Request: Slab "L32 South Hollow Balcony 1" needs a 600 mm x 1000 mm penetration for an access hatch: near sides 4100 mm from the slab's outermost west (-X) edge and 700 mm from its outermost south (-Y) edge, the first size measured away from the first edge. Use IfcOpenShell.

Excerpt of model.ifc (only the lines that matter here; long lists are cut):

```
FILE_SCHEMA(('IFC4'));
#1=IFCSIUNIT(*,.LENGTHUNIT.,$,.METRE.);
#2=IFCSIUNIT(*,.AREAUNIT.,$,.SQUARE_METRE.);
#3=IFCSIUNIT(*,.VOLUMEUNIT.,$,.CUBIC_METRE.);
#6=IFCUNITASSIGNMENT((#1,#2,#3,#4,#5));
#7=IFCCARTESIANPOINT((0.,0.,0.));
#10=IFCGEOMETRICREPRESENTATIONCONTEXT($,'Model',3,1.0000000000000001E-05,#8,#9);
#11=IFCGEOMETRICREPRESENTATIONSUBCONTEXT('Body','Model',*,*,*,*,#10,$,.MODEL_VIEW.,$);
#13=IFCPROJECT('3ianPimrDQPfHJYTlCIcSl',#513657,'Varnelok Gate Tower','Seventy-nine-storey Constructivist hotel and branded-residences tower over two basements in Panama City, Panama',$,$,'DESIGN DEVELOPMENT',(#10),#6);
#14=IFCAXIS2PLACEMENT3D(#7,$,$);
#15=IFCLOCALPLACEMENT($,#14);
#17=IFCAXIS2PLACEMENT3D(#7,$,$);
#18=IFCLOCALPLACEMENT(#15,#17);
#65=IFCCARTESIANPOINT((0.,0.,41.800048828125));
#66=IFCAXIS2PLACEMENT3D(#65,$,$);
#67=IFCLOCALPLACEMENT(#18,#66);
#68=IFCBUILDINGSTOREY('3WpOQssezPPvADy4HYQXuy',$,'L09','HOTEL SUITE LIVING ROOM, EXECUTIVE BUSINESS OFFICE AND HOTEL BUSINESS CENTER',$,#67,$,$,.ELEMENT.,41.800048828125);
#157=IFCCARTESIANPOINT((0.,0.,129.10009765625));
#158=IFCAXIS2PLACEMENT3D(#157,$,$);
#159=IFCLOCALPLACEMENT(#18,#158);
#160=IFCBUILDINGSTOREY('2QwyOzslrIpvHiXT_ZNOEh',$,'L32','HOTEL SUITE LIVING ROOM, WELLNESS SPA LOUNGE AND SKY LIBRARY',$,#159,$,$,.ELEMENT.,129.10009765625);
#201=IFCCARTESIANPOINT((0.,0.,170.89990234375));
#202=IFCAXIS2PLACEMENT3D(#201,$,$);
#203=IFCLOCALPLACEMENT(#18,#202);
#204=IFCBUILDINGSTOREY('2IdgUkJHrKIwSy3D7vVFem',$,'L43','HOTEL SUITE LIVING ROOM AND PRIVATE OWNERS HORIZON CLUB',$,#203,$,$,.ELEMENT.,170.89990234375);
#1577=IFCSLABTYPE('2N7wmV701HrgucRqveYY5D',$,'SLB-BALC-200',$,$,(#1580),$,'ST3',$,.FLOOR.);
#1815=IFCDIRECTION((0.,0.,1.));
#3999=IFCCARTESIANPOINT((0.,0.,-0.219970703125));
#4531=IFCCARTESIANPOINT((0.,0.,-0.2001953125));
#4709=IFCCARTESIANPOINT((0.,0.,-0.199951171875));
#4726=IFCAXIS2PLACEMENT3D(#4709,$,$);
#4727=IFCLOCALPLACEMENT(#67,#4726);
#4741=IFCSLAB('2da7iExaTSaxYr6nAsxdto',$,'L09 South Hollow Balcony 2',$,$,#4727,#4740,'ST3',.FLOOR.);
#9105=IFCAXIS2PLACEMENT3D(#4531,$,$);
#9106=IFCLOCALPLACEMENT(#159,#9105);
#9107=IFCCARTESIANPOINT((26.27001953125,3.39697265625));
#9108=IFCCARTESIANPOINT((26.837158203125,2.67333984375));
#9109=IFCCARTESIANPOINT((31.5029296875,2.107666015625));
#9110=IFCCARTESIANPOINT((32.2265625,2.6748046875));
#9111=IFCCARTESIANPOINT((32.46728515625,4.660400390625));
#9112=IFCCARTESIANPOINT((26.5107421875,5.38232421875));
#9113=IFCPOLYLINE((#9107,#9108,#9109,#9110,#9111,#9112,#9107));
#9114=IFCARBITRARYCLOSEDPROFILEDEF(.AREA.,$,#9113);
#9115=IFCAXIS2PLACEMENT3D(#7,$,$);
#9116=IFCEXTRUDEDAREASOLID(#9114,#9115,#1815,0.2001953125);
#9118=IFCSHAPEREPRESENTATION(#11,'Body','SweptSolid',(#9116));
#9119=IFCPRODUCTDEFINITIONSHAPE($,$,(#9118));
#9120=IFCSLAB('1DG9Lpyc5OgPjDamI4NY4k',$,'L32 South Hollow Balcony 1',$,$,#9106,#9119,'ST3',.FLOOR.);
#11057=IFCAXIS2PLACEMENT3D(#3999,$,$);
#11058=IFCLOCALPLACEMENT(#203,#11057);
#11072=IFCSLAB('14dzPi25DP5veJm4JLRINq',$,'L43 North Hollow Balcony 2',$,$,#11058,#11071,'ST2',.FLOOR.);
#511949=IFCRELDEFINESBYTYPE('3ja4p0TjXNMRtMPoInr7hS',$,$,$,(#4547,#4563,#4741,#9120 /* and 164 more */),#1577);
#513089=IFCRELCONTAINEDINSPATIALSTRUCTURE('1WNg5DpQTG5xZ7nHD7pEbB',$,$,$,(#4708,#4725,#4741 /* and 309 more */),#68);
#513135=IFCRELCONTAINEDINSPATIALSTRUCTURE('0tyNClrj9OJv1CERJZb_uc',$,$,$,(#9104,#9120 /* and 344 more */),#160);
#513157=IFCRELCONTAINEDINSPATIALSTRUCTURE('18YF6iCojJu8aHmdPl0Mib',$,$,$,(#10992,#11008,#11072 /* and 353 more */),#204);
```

```python
import numpy as np
import ifcopenshell
import ifcopenshell.api.feature
import ifcopenshell.api.geometry
import ifcopenshell.api.root
import ifcopenshell.geom
import ifcopenshell.util.placement
import ifcopenshell.util.representation
import ifcopenshell.util.shape
import ifcopenshell.util.unit

model = ifcopenshell.open("model.ifc")
unit_scale = ifcopenshell.util.unit.calculate_unit_scale(model)
settings = ifcopenshell.geom.settings()


def volume(element):
    """Net volume in cubic metres, openings subtracted."""
    shape = ifcopenshell.geom.create_shape(settings, element)
    return ifcopenshell.util.shape.get_volume(shape.geometry)


slab = model.by_guid("1DG9Lpyc5OgPjDamI4NY4k")
before = volume(slab)

# Extent in the slab's own axes, in metres. The edges named are its -X and -Y sides.
slab_shape = ifcopenshell.geom.create_shape(settings, slab)
vertices = ifcopenshell.util.shape.get_vertices(slab_shape.geometry)
x_min, y_min, bottom = vertices.min(axis=0)
top = vertices[:, 2].max()

opening = ifcopenshell.api.root.create_entity(model, ifc_class="IfcOpeningElement", name="Access hatch opening", predefined_type="OPENING")
context = ifcopenshell.util.representation.get_context(model, "Model", "Body", "MODEL_VIEW")
width, depth = 0.6, 1
outline = [(0.0, 0.0), (width, 0.0), (width, depth), (0.0, depth), (0.0, 0.0)]
# Overshoot both faces by 50 mm so the cut is clean.
shape = ifcopenshell.api.geometry.add_slab_representation(
    model, context=context, depth=top - bottom + 0.1, polyline=outline
)
ifcopenshell.api.geometry.assign_representation(model, product=opening, representation=shape)

matrix = ifcopenshell.util.placement.get_local_placement(slab.ObjectPlacement)
matrix[:, 3] = matrix @ np.append(np.array([x_min + 4.1, y_min + 0.7, bottom - 0.05]) / unit_scale, 1.0)
ifcopenshell.api.geometry.edit_object_placement(model, product=opening, matrix=matrix, is_si=False)
ifcopenshell.api.feature.add_feature(model, feature=opening, element=slab)

after = volume(slab)

print(f"slab volume {before:.3f} -> {after:.3f} m3")

model.write("model_updated.ifc")
```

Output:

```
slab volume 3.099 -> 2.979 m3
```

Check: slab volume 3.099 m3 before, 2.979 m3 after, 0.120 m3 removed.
